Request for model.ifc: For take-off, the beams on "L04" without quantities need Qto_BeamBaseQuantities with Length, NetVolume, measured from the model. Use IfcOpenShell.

First a look at what the model holds.

```python
import ifcopenshell
import ifcopenshell.util.element
import ifcopenshell.util.unit

model = ifcopenshell.open("model.ifc")
print(model.schema)
for unit_type in ("LENGTHUNIT", "AREAUNIT", "VOLUMEUNIT"):
    print(unit_type, ifcopenshell.util.unit.calculate_unit_scale(model, unit_type))
storey = next(s for s in model.by_type("IfcBuildingStorey") if s.Name == "L04")
beams = [e for e in ifcopenshell.util.element.get_decomposition(storey) if e.is_a("IfcBeam")]
for e in sorted(beams, key=lambda e: e.id()):
    print(e.id(), e.is_a(), e.Name, list(ifcopenshell.util.element.get_psets(e, qtos_only=True)), sep=" | ")
```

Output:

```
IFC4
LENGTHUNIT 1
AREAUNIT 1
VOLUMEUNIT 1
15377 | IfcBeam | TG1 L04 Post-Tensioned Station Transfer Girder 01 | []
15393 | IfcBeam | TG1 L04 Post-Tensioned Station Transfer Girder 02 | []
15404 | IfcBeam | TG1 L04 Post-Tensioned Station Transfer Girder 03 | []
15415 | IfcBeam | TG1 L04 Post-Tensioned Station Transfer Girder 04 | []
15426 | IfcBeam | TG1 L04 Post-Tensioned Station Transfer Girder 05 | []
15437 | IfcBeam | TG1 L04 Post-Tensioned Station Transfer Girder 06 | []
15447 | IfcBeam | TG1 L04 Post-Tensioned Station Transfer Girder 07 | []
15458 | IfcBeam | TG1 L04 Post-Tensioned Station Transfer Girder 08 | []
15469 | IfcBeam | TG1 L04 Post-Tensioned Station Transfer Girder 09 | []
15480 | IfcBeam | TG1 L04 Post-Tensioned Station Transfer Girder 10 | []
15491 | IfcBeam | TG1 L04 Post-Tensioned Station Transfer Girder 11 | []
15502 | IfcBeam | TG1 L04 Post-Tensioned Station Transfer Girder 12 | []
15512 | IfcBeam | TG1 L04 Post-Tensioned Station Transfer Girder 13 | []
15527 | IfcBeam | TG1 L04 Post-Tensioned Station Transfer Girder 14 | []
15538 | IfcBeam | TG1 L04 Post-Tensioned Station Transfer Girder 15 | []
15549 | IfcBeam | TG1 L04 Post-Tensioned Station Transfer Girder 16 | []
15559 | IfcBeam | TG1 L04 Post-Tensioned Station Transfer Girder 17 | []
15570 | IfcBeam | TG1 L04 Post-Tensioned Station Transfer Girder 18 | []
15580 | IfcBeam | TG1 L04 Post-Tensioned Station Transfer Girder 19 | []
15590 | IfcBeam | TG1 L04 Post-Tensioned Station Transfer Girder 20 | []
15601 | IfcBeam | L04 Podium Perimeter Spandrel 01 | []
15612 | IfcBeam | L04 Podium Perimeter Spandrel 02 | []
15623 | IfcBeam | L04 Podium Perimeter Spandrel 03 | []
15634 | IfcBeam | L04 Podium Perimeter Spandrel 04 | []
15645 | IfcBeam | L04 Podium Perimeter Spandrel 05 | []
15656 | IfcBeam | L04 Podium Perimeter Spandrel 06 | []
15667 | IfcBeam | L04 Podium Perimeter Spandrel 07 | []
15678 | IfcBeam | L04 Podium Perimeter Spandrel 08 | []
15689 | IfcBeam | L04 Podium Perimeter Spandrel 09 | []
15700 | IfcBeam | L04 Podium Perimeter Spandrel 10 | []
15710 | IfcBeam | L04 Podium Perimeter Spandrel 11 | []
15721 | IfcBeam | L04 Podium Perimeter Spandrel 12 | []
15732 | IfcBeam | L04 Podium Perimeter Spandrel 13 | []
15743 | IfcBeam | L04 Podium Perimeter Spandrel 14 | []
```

```python
import ifcopenshell
import ifcopenshell.api.pset
import ifcopenshell.geom
import ifcopenshell.util.element
import ifcopenshell.util.shape
import ifcopenshell.util.unit

model = ifcopenshell.open("model.ifc")
unit_scale = ifcopenshell.util.unit.calculate_unit_scale(model)
volume_scale = ifcopenshell.util.unit.calculate_unit_scale(model, "VOLUMEUNIT")
settings = ifcopenshell.geom.settings()

storey = next(s for s in model.by_type("IfcBuildingStorey") if s.Name == "L04")
beams = [e for e in ifcopenshell.util.element.get_decomposition(storey) if e.is_a("IfcBeam")]

for e in sorted(beams, key=lambda e: e.id()):
    if ifcopenshell.util.element.get_psets(e, qtos_only=True, should_inherit=False):
        continue
    # Geometry comes back in metres, in the element's own axes.
    shape = ifcopenshell.geom.create_shape(settings, e)
    values = {
        "Length": ifcopenshell.util.shape.get_max_xyz(shape.geometry) / unit_scale,
        "NetVolume": ifcopenshell.util.shape.get_volume(shape.geometry) / volume_scale,
    }
    qto = ifcopenshell.api.pset.add_qto(model, product=e, name="Qto_BeamBaseQuantities")
    ifcopenshell.api.pset.edit_qto(model, qto=qto, properties=values)
    print(e.id(), {k: round(v, 3) for k, v in values.items()})

model.write("model_rev.ifc")
```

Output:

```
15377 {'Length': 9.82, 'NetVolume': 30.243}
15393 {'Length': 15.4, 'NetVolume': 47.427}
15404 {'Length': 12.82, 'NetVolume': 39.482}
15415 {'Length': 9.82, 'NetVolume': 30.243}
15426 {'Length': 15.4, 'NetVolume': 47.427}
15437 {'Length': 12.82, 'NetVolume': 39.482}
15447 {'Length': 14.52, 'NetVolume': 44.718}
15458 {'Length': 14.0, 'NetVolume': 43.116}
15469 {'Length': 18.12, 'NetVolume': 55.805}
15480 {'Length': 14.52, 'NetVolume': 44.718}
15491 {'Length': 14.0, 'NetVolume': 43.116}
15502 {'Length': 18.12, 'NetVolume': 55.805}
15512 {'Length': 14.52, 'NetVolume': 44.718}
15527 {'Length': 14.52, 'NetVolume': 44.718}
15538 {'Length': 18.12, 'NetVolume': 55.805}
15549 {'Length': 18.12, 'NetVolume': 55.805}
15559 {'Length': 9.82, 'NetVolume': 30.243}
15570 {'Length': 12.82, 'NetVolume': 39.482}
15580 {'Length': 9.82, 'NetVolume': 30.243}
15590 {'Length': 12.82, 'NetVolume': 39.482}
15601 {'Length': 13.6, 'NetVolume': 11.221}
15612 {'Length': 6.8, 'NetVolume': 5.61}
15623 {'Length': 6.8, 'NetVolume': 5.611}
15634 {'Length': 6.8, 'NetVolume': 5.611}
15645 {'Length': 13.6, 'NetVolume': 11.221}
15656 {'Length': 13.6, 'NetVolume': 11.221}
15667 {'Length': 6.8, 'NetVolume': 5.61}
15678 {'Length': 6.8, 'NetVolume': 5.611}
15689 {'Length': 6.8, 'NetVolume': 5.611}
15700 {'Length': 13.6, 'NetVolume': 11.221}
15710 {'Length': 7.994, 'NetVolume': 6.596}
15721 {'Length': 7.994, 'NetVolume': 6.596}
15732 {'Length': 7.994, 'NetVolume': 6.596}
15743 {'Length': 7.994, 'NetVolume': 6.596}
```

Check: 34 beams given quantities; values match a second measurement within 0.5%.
